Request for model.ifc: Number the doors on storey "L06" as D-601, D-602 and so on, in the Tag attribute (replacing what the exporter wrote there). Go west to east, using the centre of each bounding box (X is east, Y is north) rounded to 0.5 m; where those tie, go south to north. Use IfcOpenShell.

First a look at what the model holds.

```python
import ifcopenshell
import ifcopenshell.util.element
import ifcopenshell.util.placement

model = ifcopenshell.open("model.ifc")
print(model.schema)
storey = next(s for s in model.by_type("IfcBuildingStorey") if s.Name == "L06")
doors = [e for e in ifcopenshell.util.element.get_decomposition(storey) if e.is_a("IfcDoor")]
for e in sorted(doors, key=lambda e: e.id()):
    origin = ifcopenshell.util.placement.get_local_placement(e.ObjectPlacement)[:3, 3]
    print(e.id(), e.Tag, e.Name, origin.round(2) + 0.0, sep=" | ")
```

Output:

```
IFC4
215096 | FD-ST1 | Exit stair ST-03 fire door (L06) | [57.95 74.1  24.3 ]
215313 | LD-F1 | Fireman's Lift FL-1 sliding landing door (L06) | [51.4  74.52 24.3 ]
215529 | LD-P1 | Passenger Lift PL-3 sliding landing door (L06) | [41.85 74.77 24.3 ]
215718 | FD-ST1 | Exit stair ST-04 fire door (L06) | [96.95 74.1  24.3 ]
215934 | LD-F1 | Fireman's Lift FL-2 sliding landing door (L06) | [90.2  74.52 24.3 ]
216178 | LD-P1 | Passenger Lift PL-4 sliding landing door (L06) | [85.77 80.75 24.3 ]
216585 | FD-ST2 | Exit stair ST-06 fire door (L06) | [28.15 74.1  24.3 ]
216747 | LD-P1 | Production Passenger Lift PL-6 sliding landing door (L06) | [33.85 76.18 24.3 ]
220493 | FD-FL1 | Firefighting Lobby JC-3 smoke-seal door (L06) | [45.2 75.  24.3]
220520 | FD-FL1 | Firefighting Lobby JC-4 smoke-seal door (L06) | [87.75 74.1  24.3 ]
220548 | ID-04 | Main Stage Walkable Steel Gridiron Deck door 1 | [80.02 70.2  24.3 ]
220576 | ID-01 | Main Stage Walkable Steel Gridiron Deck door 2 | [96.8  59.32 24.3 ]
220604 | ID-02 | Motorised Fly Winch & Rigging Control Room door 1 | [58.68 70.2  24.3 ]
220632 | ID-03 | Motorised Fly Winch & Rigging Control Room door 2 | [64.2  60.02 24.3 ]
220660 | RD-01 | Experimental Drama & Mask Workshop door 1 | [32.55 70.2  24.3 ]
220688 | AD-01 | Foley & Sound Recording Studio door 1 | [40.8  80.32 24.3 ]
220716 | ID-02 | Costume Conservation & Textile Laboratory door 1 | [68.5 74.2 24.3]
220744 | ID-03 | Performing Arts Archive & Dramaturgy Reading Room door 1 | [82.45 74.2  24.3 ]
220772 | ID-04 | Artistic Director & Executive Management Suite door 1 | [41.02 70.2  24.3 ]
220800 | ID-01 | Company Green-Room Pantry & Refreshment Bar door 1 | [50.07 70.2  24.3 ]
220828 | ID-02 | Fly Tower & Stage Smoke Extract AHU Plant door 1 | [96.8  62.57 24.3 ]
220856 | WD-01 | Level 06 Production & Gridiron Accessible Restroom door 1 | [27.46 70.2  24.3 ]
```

```python
import ifcopenshell
import ifcopenshell.geom
import ifcopenshell.util.element
import ifcopenshell.util.shape

model = ifcopenshell.open("model.ifc")
settings = ifcopenshell.geom.settings()
settings.set("use-world-coords", True)


def centre(element):
    shape = ifcopenshell.geom.create_shape(settings, element)
    return ifcopenshell.util.shape.get_bbox_centroid(shape.geometry)


storey = next(s for s in model.by_type("IfcBuildingStorey") if s.Name == "L06")
doors = [e for e in ifcopenshell.util.element.get_decomposition(storey) if e.is_a("IfcDoor")]

# Insertion points can sit at a corner or the storey origin, so sort by the geometry (in metres).
centres = {e: centre(e) for e in doors}
doors.sort(key=lambda e: (round(centres[e][0] / 0.5), centres[e][1]))

for i, e in enumerate(doors, start=1):
    number = f"D-6{i:02d}"
    e.Tag = number
    print(e.id(), number)

model.write("model_updated.ifc")
```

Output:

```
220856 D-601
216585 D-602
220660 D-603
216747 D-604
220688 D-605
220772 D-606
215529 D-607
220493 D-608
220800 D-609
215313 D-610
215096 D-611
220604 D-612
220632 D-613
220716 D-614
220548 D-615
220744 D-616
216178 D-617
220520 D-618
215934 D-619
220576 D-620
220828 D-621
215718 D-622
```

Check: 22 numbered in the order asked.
